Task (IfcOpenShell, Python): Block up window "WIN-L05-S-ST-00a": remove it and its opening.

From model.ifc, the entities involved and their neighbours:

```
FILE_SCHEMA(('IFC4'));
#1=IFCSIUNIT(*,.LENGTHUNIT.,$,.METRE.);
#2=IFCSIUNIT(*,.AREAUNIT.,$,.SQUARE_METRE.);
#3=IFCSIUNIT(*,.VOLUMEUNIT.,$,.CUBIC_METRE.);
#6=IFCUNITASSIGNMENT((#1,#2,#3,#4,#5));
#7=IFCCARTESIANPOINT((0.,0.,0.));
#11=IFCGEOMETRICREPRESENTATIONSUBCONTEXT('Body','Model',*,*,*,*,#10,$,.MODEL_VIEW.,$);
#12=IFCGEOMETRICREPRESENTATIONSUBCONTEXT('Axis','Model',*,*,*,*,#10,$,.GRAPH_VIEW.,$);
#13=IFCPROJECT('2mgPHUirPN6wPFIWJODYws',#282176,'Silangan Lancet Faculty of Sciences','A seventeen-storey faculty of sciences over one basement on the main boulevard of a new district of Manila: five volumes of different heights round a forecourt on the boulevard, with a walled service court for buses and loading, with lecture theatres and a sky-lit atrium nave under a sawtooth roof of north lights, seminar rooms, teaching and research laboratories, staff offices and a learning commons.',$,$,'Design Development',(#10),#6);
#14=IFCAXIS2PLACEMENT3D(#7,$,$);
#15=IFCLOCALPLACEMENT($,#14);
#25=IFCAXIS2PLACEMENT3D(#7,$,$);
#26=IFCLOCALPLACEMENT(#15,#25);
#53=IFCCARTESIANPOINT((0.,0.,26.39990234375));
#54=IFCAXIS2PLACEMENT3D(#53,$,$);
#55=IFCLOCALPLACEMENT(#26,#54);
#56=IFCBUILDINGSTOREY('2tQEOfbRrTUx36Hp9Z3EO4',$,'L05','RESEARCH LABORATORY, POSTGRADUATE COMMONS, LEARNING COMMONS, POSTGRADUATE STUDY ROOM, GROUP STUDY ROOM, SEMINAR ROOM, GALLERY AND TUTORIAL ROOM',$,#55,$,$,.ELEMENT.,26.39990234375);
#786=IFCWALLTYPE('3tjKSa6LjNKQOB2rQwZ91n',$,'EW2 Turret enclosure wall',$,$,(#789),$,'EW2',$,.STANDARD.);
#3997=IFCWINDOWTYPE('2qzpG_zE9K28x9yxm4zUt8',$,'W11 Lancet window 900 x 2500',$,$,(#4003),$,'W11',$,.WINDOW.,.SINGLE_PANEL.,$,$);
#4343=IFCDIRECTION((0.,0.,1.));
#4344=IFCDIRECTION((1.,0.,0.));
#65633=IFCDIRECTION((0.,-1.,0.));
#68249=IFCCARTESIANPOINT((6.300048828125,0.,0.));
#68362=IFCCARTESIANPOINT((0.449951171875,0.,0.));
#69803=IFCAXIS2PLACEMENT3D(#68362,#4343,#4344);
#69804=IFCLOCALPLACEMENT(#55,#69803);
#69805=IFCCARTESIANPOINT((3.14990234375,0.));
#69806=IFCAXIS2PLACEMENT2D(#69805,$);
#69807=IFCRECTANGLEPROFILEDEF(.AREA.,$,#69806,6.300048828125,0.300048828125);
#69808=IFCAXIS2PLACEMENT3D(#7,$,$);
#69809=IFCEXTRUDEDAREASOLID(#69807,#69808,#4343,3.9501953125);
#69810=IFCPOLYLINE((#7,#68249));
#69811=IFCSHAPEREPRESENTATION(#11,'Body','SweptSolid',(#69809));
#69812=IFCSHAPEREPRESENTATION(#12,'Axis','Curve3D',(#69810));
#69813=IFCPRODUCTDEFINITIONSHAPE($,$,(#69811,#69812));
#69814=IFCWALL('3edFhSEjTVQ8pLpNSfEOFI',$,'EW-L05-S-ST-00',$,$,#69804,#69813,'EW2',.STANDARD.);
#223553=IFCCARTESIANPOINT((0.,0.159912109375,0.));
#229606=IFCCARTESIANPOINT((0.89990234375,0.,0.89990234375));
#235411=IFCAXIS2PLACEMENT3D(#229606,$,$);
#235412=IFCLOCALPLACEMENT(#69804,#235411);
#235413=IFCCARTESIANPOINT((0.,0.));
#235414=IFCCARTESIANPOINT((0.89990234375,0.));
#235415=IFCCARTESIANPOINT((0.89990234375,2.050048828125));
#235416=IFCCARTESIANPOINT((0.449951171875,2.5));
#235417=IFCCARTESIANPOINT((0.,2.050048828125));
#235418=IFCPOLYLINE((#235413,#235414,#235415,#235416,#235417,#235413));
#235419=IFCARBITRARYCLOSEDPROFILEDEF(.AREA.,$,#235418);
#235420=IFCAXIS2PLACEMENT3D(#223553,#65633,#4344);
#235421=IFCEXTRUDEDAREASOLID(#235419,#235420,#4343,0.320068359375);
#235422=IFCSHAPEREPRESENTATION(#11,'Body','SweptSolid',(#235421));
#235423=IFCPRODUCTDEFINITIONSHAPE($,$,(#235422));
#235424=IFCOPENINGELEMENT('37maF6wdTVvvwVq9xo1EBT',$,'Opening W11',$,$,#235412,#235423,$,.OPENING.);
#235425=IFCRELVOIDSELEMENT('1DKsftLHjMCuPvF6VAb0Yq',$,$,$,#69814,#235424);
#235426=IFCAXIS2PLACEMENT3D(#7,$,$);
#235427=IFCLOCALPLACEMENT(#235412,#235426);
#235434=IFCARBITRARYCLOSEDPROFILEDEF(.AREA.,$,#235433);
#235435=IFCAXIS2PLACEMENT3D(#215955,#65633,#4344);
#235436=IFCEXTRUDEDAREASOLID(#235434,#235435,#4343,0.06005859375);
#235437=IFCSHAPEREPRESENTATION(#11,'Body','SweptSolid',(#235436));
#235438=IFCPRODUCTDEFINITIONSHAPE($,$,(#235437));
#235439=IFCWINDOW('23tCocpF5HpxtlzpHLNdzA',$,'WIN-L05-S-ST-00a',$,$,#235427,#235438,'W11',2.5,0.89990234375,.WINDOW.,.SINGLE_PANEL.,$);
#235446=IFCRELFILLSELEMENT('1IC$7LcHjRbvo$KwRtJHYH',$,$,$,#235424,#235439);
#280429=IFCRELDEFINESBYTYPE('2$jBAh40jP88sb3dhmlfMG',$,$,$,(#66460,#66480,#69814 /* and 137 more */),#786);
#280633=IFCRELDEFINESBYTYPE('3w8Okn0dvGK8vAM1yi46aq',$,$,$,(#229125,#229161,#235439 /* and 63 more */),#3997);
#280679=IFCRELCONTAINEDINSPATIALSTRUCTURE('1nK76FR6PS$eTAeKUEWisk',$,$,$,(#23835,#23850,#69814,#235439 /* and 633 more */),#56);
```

```python
import ifcopenshell
import ifcopenshell.api.feature
import ifcopenshell.api.root
import ifcopenshell.geom
import ifcopenshell.util.shape

model = ifcopenshell.open("model.ifc")
settings = ifcopenshell.geom.settings()


def volume(element):
    """Net volume in cubic metres, openings subtracted."""
    shape = ifcopenshell.geom.create_shape(settings, element)
    return ifcopenshell.util.shape.get_volume(shape.geometry)


window = model.by_guid("23tCocpF5HpxtlzpHLNdzA")
opening = window.FillsVoids[0].RelatingOpeningElement
wall = opening.VoidsElements[0].RelatingBuildingElement
before = volume(wall)

ifcopenshell.api.root.remove_product(model, product=window)
ifcopenshell.api.feature.remove_feature(model, feature=opening)

after = volume(wall)

print(f"wall volume {before:.3f} -> {after:.3f} m3")

model.write("model_edited.ifc")
```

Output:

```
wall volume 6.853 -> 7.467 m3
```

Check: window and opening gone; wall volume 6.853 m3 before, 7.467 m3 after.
